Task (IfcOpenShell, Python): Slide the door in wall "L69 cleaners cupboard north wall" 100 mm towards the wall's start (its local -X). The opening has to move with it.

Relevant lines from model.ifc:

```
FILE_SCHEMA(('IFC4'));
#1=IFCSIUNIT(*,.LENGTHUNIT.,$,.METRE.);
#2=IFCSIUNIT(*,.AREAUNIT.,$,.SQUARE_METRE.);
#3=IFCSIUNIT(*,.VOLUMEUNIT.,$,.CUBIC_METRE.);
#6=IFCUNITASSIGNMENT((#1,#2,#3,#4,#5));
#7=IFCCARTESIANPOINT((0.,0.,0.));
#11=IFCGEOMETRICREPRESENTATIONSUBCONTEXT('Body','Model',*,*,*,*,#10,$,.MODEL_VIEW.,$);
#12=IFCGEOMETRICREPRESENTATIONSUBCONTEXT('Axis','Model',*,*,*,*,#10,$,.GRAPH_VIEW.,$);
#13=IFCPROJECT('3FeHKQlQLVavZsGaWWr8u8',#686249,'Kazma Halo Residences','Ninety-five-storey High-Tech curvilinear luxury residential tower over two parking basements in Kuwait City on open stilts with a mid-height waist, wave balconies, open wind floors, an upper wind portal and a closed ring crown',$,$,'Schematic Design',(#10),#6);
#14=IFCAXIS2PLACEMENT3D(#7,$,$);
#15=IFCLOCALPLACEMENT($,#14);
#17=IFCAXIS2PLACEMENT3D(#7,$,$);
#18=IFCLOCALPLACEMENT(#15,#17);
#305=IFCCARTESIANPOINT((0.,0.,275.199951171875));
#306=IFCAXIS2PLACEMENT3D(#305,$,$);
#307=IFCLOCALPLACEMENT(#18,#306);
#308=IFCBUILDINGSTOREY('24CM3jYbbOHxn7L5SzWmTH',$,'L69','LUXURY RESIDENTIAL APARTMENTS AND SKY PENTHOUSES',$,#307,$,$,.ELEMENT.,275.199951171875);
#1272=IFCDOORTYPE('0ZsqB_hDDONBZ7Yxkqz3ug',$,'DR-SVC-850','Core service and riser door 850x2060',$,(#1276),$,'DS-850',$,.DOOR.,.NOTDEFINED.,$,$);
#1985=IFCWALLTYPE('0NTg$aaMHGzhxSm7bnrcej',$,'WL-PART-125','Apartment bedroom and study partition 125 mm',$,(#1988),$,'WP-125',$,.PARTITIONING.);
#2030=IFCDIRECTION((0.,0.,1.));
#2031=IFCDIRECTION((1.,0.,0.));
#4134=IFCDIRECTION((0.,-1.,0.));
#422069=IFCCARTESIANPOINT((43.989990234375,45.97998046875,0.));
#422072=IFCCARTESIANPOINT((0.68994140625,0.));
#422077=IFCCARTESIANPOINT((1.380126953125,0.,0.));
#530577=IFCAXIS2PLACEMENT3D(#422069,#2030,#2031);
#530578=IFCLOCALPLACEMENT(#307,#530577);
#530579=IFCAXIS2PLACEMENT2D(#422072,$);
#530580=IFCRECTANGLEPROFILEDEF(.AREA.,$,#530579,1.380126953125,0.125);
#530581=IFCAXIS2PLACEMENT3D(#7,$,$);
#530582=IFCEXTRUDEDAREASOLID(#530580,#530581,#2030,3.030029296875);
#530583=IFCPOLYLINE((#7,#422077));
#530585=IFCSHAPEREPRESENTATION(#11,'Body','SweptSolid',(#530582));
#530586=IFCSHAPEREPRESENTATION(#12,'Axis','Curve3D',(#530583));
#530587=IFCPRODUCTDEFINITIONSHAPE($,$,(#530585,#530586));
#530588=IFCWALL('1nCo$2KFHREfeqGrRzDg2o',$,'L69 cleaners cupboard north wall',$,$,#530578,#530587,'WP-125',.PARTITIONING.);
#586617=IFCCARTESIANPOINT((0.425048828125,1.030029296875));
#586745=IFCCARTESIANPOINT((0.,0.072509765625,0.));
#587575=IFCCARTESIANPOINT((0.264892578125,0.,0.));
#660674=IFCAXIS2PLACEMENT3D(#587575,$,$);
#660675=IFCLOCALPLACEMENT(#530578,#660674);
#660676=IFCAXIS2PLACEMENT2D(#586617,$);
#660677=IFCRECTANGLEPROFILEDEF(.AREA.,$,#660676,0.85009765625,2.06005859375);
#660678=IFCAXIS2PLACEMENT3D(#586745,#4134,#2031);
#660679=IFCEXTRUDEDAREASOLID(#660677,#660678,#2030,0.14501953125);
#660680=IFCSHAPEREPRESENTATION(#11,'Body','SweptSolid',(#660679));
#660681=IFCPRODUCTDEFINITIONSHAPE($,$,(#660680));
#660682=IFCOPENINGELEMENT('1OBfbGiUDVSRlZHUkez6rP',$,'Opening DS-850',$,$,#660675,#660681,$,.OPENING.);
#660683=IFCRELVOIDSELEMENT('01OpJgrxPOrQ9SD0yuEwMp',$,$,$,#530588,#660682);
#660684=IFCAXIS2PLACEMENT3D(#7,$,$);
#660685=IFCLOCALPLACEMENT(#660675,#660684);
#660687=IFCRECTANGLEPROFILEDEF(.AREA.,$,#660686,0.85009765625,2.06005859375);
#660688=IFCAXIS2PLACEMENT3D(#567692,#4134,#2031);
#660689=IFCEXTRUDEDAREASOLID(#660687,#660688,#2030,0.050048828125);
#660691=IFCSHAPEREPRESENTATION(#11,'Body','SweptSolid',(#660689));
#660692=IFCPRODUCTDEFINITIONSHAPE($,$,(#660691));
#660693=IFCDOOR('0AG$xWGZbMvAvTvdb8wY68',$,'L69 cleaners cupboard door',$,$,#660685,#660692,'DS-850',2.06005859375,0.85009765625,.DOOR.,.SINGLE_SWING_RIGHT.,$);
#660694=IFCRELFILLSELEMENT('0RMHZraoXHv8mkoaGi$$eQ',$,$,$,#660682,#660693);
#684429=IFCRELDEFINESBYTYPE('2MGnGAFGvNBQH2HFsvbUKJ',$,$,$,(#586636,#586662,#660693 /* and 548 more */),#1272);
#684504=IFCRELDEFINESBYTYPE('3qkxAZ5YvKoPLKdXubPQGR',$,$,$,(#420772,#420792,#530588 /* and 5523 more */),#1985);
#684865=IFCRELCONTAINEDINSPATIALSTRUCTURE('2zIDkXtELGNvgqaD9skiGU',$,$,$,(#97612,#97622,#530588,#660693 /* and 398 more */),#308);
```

```python
import ifcopenshell
import ifcopenshell.api.geometry
import ifcopenshell.util.placement
import ifcopenshell.util.unit

model = ifcopenshell.open("model.ifc")
unit_scale = ifcopenshell.util.unit.calculate_unit_scale(model)

door = model.by_guid("0AG$xWGZbMvAvTvdb8wY68")
opening = door.FillsVoids[0].RelatingOpeningElement
wall = opening.VoidsElements[0].RelatingBuildingElement

wall_matrix = ifcopenshell.util.placement.get_local_placement(wall.ObjectPlacement)
shift = wall_matrix[:3, 0] * -0.1 / unit_scale
before = ifcopenshell.util.placement.get_local_placement(door.ObjectPlacement)[:3, 3].copy()

# The door is placed relative to its opening, so it follows when the opening moves.
matrix = ifcopenshell.util.placement.get_local_placement(opening.ObjectPlacement)
matrix[:3, 3] += shift
ifcopenshell.api.geometry.edit_object_placement(
    model, product=opening, matrix=matrix, is_si=False, should_transform_children=True
)

after = ifcopenshell.util.placement.get_local_placement(door.ObjectPlacement)[:3, 3]
print("door moved by", (after - before).round(3) + 0.0)

model.write("model-out.ifc")
```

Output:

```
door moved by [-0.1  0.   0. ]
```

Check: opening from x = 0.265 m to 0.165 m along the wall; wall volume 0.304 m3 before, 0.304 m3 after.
